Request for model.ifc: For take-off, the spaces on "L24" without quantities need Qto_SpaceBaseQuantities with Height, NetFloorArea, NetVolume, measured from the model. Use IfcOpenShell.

First a look at what the model holds.

```python
import ifcopenshell
import ifcopenshell.util.element
import ifcopenshell.util.unit

model = ifcopenshell.open("model.ifc")
print(model.schema)
for unit_type in ("LENGTHUNIT", "AREAUNIT", "VOLUMEUNIT"):
    print(unit_type, ifcopenshell.util.unit.calculate_unit_scale(model, unit_type))
storey = next(s for s in model.by_type("IfcBuildingStorey") if s.Name == "L24")
spaces = [e for e in ifcopenshell.util.element.get_decomposition(storey) if e.is_a("IfcSpace")]
for e in sorted(spaces, key=lambda e: e.id()):
    print(e.id(), e.is_a(), e.Name, list(ifcopenshell.util.element.get_psets(e, qtos_only=True)), sep=" | ")
```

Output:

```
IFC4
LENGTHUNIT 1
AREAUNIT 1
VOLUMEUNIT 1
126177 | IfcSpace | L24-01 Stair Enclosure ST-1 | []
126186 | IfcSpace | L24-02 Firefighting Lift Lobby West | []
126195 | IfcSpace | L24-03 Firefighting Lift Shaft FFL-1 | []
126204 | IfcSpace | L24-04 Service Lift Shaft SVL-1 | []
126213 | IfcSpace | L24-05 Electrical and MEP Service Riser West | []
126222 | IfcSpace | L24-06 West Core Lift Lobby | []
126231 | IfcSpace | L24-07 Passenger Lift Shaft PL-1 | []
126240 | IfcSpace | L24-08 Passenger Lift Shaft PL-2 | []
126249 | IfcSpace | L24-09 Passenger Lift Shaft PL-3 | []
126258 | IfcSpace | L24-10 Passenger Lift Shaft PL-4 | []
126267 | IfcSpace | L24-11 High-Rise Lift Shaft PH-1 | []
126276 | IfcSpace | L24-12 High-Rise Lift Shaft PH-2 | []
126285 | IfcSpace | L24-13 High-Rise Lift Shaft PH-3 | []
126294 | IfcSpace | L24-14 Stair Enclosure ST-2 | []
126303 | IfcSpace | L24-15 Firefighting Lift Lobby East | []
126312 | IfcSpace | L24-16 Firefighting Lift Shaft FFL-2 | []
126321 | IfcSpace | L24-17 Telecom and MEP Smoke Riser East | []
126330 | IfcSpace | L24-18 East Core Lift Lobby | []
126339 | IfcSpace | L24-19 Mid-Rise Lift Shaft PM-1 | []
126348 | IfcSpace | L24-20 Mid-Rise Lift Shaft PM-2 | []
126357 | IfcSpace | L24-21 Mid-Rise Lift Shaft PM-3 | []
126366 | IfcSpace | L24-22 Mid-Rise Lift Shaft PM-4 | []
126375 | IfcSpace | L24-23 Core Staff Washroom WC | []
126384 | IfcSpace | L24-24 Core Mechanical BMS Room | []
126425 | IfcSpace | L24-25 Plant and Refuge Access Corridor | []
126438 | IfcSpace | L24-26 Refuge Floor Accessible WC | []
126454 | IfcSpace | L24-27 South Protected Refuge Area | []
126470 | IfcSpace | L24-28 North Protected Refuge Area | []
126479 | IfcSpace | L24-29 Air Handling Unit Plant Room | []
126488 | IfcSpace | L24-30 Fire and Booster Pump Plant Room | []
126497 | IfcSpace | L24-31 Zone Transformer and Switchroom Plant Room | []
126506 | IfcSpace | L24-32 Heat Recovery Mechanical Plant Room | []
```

```python
import ifcopenshell
import ifcopenshell.api.pset
import ifcopenshell.geom
import ifcopenshell.util.element
import ifcopenshell.util.shape
import ifcopenshell.util.unit

model = ifcopenshell.open("model.ifc")
unit_scale = ifcopenshell.util.unit.calculate_unit_scale(model)
area_scale = ifcopenshell.util.unit.calculate_unit_scale(model, "AREAUNIT")
volume_scale = ifcopenshell.util.unit.calculate_unit_scale(model, "VOLUMEUNIT")
settings = ifcopenshell.geom.settings()

storey = next(s for s in model.by_type("IfcBuildingStorey") if s.Name == "L24")
spaces = [e for e in ifcopenshell.util.element.get_decomposition(storey) if e.is_a("IfcSpace")]

for e in sorted(spaces, key=lambda e: e.id()):
    if ifcopenshell.util.element.get_psets(e, qtos_only=True, should_inherit=False):
        continue
    # Geometry comes back in metres, in the element's own axes.
    shape = ifcopenshell.geom.create_shape(settings, e)
    values = {
        "Height": ifcopenshell.util.shape.get_z(shape.geometry) / unit_scale,
        "NetFloorArea": ifcopenshell.util.shape.get_footprint_area(shape.geometry) / area_scale,
        "NetVolume": ifcopenshell.util.shape.get_volume(shape.geometry) / volume_scale,
    }
    qto = ifcopenshell.api.pset.add_qto(model, product=e, name="Qto_SpaceBaseQuantities")
    ifcopenshell.api.pset.edit_qto(model, qto=qto, properties=values)
    print(e.id(), {k: round(v, 3) for k, v in values.items()})

model.write("model_updated.ifc")
```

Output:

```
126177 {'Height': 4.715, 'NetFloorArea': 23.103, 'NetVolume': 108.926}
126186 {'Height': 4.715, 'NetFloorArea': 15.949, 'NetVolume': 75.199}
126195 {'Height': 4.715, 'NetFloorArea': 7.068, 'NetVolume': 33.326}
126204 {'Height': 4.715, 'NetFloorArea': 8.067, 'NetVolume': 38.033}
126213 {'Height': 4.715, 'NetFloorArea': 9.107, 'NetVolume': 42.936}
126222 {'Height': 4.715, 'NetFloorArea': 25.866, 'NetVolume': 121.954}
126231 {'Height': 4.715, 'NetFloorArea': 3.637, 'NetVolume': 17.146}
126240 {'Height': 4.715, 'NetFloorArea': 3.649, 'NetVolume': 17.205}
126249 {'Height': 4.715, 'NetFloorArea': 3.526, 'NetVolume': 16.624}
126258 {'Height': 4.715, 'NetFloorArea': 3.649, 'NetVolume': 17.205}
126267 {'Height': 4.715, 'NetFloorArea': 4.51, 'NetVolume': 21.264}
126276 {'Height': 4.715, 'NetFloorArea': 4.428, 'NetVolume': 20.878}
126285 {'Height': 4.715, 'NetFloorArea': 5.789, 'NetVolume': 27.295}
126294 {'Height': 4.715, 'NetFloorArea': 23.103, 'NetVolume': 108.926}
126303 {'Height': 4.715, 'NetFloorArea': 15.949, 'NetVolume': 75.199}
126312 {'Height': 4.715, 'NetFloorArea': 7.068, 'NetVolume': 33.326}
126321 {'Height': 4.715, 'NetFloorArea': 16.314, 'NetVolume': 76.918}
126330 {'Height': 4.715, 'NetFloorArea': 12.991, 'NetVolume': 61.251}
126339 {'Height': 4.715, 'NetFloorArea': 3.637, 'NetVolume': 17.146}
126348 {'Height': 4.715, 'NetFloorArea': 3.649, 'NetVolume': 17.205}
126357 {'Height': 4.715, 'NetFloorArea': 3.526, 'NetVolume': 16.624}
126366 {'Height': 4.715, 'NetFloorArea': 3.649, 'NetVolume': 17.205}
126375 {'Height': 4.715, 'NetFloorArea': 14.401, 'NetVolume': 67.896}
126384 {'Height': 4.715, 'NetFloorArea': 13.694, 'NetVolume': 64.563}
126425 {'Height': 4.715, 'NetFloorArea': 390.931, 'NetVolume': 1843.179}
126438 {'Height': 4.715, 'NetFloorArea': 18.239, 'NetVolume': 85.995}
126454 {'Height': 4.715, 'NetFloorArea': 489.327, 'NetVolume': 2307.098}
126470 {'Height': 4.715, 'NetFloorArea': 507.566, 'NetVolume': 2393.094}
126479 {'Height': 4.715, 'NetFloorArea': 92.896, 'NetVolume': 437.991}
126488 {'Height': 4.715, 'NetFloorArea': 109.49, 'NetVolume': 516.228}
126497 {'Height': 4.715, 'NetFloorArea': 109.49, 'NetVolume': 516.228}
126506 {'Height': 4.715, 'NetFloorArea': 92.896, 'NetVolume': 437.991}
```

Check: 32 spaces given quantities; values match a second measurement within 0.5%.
